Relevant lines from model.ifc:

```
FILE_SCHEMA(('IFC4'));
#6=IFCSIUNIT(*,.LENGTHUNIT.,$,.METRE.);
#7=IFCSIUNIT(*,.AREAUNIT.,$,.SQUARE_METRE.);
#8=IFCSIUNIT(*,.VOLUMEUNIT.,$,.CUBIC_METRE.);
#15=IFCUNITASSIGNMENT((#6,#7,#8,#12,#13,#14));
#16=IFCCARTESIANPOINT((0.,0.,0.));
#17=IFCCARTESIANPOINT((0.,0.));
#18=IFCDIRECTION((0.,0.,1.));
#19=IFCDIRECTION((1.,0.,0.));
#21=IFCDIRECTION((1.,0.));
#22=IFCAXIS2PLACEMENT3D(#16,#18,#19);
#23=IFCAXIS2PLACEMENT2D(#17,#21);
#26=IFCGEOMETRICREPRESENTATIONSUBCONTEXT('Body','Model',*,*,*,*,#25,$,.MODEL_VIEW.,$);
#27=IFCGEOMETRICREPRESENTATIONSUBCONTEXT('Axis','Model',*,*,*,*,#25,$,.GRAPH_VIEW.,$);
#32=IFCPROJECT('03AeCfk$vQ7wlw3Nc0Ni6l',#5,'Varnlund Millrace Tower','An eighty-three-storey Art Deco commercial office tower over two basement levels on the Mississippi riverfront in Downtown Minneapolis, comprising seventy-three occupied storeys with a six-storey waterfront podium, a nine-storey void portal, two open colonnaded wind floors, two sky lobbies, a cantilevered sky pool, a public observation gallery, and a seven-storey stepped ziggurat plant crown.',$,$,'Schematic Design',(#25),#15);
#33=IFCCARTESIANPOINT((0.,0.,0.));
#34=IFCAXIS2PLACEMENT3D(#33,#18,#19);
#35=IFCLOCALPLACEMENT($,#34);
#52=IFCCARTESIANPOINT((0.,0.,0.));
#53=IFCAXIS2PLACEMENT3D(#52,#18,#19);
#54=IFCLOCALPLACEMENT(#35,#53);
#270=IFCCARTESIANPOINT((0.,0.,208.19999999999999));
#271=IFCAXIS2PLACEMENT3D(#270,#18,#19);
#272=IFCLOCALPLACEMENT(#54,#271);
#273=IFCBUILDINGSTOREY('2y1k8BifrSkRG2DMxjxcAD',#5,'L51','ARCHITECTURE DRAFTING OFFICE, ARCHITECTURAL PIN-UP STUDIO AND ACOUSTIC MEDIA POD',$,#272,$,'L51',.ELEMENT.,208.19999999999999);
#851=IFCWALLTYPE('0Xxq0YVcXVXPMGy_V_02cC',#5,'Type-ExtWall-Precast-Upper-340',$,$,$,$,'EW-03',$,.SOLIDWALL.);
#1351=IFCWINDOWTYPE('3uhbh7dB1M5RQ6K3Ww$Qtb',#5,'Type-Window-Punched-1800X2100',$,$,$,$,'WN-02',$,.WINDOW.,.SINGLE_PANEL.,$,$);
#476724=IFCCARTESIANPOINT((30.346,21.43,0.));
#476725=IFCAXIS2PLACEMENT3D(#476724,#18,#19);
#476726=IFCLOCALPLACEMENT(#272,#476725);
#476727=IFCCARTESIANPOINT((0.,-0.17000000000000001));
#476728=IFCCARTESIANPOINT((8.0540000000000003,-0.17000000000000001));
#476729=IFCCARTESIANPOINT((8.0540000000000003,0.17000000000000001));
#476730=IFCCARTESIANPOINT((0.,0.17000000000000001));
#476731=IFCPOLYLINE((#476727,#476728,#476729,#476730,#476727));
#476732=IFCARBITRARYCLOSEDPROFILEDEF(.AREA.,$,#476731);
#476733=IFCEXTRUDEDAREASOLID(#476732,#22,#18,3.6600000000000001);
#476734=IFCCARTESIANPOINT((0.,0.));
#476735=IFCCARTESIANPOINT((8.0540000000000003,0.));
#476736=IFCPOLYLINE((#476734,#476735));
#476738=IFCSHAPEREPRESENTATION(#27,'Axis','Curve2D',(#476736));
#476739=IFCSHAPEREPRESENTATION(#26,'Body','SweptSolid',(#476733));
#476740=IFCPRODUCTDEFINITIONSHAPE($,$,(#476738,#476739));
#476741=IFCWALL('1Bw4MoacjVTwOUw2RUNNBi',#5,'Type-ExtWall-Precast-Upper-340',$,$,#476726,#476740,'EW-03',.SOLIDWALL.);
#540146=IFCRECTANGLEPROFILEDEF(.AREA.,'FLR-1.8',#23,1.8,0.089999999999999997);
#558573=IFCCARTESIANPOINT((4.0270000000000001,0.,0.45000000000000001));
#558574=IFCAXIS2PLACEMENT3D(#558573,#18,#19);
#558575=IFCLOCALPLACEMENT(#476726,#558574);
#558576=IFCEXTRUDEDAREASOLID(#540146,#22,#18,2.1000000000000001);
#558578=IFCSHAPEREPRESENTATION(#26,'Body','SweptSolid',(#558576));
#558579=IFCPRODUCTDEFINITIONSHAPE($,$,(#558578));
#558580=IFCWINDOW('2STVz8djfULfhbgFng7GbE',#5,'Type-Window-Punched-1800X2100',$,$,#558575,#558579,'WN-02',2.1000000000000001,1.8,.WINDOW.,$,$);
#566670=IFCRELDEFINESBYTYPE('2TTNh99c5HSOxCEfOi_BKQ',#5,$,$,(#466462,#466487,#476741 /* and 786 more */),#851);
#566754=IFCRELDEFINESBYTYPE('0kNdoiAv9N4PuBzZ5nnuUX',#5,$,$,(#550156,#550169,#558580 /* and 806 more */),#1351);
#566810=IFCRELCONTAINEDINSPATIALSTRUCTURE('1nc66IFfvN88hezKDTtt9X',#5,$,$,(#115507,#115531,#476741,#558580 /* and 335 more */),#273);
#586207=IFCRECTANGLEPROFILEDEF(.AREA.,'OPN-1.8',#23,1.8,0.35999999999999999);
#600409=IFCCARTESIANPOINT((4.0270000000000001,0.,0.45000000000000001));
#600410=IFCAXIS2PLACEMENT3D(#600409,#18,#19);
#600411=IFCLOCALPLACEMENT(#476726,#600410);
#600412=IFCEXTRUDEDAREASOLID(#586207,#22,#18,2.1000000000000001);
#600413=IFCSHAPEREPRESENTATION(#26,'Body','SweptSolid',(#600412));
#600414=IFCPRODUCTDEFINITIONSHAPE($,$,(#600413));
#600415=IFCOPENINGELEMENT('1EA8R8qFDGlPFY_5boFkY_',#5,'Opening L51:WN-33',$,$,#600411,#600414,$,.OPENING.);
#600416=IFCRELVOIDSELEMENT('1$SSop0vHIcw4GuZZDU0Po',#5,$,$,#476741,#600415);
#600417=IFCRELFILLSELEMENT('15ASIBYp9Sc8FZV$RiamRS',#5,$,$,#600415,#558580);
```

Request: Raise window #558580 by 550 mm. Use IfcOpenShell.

```python
import numpy as np
import ifcopenshell
import ifcopenshell.api.geometry
import ifcopenshell.util.placement
import ifcopenshell.util.unit

model = ifcopenshell.open("model.ifc")
unit_scale = ifcopenshell.util.unit.calculate_unit_scale(model)

window = model.by_guid("2STVz8djfULfhbgFng7GbE")
opening = window.FillsVoids[0].RelatingOpeningElement
dz = 0.55

shift = np.array([0.0, 0.0, dz])
# The window is not placed relative to its opening, so move both.
for product in (opening, window):
    matrix = ifcopenshell.util.placement.get_local_placement(product.ObjectPlacement)
    matrix[:3, 3] += shift
    ifcopenshell.api.geometry.edit_object_placement(model, product=product, matrix=matrix, is_si=False)

print(f"moved by {dz * unit_scale:+.3f} m")

model.write("model_v2.ifc")
```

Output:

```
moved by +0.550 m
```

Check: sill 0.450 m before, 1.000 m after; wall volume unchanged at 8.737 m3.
